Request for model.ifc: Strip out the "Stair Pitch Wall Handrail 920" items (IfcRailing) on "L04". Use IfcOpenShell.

First a look at what the model holds.

```python
import ifcopenshell
import ifcopenshell.util.element

model = ifcopenshell.open("model.ifc")
print(model.schema)
storey = next(s for s in model.by_type("IfcBuildingStorey") if s.Name == "L04")
railings = [e for e in ifcopenshell.util.element.get_decomposition(storey) if e.is_a("IfcRailing")]
seen = {}
for e in railings:
    element_type = ifcopenshell.util.element.get_type(e)
    name = element_type.Name if element_type not in (None, e) else None
    seen[name] = seen.get(name, 0) + 1
for name, count in sorted(seen.items(), key=str):
    print(count, "x", name)
```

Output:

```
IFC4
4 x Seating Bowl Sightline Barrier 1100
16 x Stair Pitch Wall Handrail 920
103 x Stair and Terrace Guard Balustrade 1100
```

```python
import ifcopenshell
import ifcopenshell.api.root
import ifcopenshell.util.element

model = ifcopenshell.open("model.ifc")

storey = next(s for s in model.by_type("IfcBuildingStorey") if s.Name == "L04")
railings = [e for e in ifcopenshell.util.element.get_decomposition(storey) if e.is_a("IfcRailing")]
targets = [e for e in railings if (t := ifcopenshell.util.element.get_type(e)) not in (None, e) and t.Name == "Stair Pitch Wall Handrail 920"]

for e in targets:
    ifcopenshell.api.root.remove_product(model, product=e)
print(len(targets), "removed")

model.write("model_updated.ifc")
```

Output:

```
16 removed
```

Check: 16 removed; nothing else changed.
